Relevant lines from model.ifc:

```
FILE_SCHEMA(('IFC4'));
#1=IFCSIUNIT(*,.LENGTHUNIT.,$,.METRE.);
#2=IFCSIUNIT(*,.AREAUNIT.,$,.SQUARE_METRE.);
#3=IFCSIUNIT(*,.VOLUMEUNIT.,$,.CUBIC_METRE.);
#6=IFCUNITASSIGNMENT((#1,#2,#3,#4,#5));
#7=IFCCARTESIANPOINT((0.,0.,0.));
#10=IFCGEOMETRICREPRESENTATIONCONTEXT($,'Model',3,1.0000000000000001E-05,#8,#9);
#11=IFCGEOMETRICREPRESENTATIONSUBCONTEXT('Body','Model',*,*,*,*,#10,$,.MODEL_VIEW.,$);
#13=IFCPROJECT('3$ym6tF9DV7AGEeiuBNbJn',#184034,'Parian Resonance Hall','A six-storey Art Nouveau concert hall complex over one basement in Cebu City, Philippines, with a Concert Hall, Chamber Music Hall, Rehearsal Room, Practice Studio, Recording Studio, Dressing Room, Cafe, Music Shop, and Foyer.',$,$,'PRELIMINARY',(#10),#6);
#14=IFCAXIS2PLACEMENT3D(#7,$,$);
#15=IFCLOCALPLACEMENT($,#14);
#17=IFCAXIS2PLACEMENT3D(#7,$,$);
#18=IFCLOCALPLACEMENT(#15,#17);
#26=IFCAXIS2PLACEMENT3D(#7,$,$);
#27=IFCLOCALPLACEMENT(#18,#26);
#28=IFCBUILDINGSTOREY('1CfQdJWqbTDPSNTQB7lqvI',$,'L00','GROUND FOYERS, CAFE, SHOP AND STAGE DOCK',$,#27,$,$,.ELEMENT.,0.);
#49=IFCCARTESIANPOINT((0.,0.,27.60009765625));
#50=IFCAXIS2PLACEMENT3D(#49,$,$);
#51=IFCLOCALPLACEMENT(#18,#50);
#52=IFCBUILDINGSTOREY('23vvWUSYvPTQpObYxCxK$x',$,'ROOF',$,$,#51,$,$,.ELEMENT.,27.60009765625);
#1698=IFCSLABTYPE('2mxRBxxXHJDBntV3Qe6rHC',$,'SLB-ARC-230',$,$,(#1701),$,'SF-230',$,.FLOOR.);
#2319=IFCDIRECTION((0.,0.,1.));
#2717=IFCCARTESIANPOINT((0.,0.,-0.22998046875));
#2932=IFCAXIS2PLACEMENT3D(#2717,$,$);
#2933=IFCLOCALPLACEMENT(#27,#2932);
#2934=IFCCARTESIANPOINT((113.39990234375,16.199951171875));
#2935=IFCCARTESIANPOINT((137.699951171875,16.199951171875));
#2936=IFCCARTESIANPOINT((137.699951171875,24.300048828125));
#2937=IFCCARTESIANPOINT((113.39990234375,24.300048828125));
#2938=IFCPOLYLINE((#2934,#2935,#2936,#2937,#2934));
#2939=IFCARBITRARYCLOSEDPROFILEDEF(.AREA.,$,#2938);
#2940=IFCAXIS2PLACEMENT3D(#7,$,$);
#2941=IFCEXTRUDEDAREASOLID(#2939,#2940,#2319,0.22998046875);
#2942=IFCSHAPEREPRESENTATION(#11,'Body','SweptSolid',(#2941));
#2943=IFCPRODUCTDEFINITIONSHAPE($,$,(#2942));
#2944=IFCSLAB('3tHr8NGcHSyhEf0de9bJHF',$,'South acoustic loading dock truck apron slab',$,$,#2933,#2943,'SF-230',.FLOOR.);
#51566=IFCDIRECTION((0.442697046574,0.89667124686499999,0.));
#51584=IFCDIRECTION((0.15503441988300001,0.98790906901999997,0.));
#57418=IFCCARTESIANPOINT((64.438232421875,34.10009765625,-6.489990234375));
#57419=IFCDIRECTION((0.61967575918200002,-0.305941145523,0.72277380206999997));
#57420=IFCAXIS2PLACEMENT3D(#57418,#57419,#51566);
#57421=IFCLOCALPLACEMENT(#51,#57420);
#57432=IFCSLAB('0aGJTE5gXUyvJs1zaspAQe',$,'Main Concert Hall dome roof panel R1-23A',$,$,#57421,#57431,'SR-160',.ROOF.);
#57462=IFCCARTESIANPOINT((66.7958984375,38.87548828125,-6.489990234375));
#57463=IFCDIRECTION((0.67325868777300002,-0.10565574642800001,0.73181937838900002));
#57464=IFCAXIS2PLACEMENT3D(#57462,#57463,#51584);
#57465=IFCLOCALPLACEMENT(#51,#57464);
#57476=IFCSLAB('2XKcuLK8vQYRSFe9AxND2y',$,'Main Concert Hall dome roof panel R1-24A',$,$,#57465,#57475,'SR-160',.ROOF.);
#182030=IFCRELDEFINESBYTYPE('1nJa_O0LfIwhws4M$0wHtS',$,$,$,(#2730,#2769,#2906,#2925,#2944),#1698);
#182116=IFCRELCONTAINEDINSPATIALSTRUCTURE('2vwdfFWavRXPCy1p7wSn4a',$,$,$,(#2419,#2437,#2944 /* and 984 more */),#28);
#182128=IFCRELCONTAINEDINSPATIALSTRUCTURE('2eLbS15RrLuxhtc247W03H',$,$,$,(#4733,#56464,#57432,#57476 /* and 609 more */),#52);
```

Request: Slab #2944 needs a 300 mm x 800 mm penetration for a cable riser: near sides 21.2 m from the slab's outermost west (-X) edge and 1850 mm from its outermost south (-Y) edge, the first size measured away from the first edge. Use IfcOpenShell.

```python
import numpy as np
import ifcopenshell
import ifcopenshell.api.feature
import ifcopenshell.api.geometry
import ifcopenshell.api.root
import ifcopenshell.geom
import ifcopenshell.util.placement
import ifcopenshell.util.representation
import ifcopenshell.util.shape
import ifcopenshell.util.unit

model = ifcopenshell.open("model.ifc")
unit_scale = ifcopenshell.util.unit.calculate_unit_scale(model)
settings = ifcopenshell.geom.settings()


def volume(element):
    """Net volume in cubic metres, openings subtracted."""
    shape = ifcopenshell.geom.create_shape(settings, element)
    return ifcopenshell.util.shape.get_volume(shape.geometry)


slab = model.by_guid("3tHr8NGcHSyhEf0de9bJHF")
before = volume(slab)

# Extent in the slab's own axes, in metres. The edges named are its -X and -Y sides.
slab_shape = ifcopenshell.geom.create_shape(settings, slab)
vertices = ifcopenshell.util.shape.get_vertices(slab_shape.geometry)
x_min, y_min, bottom = vertices.min(axis=0)
top = vertices[:, 2].max()

opening = ifcopenshell.api.root.create_entity(model, ifc_class="IfcOpeningElement", name="Cable riser opening", predefined_type="OPENING")
context = ifcopenshell.util.representation.get_context(model, "Model", "Body", "MODEL_VIEW")
width, depth = 0.3, 0.8
outline = [(0.0, 0.0), (width, 0.0), (width, depth), (0.0, depth), (0.0, 0.0)]
# Overshoot both faces by 50 mm so the cut is clean.
shape = ifcopenshell.api.geometry.add_slab_representation(
    model, context=context, depth=top - bottom + 0.1, polyline=outline
)
ifcopenshell.api.geometry.assign_representation(model, product=opening, representation=shape)

matrix = ifcopenshell.util.placement.get_local_placement(slab.ObjectPlacement)
matrix[:, 3] = matrix @ np.append(np.array([x_min + 21.2, y_min + 1.85, bottom - 0.05]) / unit_scale, 1.0)
ifcopenshell.api.geometry.edit_object_placement(model, product=opening, matrix=matrix, is_si=False)
ifcopenshell.api.feature.add_feature(model, feature=opening, element=slab)

after = volume(slab)

print(f"slab volume {before:.3f} -> {after:.3f} m3")

model.write("model_updated.ifc")
```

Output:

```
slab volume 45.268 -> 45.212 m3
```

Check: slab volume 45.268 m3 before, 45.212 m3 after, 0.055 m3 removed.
